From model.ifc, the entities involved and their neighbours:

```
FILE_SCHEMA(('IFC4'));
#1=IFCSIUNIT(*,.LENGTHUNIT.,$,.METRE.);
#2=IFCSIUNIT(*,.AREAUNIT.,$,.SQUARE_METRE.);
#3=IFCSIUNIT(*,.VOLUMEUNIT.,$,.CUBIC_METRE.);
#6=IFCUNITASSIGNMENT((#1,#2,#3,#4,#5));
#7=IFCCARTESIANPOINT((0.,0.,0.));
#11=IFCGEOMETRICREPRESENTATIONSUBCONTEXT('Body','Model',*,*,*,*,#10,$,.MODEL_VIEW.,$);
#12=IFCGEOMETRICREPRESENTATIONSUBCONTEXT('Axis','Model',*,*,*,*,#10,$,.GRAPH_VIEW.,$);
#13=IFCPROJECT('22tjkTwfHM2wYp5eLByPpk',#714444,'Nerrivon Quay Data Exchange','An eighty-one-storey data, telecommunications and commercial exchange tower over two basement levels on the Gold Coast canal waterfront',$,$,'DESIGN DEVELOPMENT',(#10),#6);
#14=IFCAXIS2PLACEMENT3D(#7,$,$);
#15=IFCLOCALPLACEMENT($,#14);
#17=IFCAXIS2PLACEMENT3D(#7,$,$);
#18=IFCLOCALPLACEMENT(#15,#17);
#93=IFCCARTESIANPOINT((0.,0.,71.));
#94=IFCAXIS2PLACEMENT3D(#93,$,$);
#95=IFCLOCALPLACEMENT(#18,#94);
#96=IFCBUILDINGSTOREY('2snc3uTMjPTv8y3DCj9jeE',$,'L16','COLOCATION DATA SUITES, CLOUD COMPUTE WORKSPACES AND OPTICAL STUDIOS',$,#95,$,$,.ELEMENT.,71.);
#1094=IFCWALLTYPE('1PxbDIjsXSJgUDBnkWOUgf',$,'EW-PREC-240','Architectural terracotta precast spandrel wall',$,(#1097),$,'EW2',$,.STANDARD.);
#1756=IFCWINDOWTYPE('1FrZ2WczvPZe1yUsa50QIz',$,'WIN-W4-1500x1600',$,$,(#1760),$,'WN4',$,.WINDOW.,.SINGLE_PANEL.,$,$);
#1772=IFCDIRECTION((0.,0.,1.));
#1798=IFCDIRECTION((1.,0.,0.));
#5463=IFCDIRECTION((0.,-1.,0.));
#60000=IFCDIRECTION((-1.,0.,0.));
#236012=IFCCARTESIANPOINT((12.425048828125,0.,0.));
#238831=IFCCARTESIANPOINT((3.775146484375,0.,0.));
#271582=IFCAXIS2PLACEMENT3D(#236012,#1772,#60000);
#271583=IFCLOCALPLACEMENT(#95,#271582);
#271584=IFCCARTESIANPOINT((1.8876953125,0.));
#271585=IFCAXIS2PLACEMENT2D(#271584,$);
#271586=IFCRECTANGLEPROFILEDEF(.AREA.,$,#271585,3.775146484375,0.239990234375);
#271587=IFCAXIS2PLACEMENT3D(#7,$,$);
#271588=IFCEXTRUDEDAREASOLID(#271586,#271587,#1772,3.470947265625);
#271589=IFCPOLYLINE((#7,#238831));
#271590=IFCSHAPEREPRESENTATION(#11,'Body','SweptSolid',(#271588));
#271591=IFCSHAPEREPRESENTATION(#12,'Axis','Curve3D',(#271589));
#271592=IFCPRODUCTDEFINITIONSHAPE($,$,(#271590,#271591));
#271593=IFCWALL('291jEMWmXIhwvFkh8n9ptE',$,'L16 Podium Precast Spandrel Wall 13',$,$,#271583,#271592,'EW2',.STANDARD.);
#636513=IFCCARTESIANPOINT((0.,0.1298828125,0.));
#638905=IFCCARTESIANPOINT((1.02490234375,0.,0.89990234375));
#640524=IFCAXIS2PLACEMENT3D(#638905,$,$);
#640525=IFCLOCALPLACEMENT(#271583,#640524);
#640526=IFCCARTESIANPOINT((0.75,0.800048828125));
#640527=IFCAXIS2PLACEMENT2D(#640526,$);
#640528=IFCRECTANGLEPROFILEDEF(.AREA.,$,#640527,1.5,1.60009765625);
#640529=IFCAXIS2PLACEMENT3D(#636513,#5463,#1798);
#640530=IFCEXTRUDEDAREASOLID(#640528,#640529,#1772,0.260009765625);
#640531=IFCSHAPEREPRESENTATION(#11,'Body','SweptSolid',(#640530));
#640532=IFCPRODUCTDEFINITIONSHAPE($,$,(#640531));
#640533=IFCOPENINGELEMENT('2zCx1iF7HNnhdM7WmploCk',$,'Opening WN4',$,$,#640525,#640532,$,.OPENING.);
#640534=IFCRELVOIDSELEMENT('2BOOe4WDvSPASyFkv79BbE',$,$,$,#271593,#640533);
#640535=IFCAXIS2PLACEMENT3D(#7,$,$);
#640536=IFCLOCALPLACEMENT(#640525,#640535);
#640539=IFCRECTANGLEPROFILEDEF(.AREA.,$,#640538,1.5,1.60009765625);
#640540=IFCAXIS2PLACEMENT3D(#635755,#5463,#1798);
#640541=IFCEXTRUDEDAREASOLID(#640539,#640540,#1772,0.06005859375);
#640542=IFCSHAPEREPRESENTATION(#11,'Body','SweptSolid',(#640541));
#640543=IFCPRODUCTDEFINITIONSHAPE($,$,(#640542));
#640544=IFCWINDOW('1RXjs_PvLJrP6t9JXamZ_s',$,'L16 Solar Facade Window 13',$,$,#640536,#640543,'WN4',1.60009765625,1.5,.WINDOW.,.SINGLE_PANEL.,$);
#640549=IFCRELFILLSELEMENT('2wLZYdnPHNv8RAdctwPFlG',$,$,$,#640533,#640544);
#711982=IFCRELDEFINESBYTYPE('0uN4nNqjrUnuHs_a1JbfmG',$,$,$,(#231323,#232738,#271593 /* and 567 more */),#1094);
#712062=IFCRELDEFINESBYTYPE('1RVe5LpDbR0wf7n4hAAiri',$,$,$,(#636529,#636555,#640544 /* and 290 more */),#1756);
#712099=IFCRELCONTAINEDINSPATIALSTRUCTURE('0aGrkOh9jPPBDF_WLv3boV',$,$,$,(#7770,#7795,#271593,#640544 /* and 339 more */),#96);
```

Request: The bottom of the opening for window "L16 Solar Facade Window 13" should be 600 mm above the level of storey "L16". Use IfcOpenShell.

```python
import numpy as np
import ifcopenshell
import ifcopenshell.api.geometry
import ifcopenshell.geom
import ifcopenshell.util.element
import ifcopenshell.util.placement
import ifcopenshell.util.shape
import ifcopenshell.util.unit

model = ifcopenshell.open("model.ifc")
unit_scale = ifcopenshell.util.unit.calculate_unit_scale(model)

window = model.by_guid("1RXjs_PvLJrP6t9JXamZ_s")
opening = window.FillsVoids[0].RelatingOpeningElement
storey = ifcopenshell.util.element.get_container(window, ifc_class="IfcBuildingStorey")
level = ifcopenshell.util.placement.get_local_placement(storey.ObjectPlacement)[2, 3]

# The opening's origin need not be at the sill, so measure its lowest point.
shape = ifcopenshell.geom.create_shape(ifcopenshell.geom.settings(), opening)
bottom = ifcopenshell.util.shape.get_shape_bottom_elevation(shape, shape.geometry) / unit_scale
dz = level + 0.6 / unit_scale - bottom

shift = np.array([0.0, 0.0, dz])
# The window is placed relative to its opening, so it follows when the opening moves.
matrix = ifcopenshell.util.placement.get_local_placement(opening.ObjectPlacement)
matrix[:3, 3] += shift
ifcopenshell.api.geometry.edit_object_placement(
    model, product=opening, matrix=matrix, is_si=False, should_transform_children=True
)

print(f"moved by {dz * unit_scale:+.3f} m")

model.write("model_rev.ifc")
```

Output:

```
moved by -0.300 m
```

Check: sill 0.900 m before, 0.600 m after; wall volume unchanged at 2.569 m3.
